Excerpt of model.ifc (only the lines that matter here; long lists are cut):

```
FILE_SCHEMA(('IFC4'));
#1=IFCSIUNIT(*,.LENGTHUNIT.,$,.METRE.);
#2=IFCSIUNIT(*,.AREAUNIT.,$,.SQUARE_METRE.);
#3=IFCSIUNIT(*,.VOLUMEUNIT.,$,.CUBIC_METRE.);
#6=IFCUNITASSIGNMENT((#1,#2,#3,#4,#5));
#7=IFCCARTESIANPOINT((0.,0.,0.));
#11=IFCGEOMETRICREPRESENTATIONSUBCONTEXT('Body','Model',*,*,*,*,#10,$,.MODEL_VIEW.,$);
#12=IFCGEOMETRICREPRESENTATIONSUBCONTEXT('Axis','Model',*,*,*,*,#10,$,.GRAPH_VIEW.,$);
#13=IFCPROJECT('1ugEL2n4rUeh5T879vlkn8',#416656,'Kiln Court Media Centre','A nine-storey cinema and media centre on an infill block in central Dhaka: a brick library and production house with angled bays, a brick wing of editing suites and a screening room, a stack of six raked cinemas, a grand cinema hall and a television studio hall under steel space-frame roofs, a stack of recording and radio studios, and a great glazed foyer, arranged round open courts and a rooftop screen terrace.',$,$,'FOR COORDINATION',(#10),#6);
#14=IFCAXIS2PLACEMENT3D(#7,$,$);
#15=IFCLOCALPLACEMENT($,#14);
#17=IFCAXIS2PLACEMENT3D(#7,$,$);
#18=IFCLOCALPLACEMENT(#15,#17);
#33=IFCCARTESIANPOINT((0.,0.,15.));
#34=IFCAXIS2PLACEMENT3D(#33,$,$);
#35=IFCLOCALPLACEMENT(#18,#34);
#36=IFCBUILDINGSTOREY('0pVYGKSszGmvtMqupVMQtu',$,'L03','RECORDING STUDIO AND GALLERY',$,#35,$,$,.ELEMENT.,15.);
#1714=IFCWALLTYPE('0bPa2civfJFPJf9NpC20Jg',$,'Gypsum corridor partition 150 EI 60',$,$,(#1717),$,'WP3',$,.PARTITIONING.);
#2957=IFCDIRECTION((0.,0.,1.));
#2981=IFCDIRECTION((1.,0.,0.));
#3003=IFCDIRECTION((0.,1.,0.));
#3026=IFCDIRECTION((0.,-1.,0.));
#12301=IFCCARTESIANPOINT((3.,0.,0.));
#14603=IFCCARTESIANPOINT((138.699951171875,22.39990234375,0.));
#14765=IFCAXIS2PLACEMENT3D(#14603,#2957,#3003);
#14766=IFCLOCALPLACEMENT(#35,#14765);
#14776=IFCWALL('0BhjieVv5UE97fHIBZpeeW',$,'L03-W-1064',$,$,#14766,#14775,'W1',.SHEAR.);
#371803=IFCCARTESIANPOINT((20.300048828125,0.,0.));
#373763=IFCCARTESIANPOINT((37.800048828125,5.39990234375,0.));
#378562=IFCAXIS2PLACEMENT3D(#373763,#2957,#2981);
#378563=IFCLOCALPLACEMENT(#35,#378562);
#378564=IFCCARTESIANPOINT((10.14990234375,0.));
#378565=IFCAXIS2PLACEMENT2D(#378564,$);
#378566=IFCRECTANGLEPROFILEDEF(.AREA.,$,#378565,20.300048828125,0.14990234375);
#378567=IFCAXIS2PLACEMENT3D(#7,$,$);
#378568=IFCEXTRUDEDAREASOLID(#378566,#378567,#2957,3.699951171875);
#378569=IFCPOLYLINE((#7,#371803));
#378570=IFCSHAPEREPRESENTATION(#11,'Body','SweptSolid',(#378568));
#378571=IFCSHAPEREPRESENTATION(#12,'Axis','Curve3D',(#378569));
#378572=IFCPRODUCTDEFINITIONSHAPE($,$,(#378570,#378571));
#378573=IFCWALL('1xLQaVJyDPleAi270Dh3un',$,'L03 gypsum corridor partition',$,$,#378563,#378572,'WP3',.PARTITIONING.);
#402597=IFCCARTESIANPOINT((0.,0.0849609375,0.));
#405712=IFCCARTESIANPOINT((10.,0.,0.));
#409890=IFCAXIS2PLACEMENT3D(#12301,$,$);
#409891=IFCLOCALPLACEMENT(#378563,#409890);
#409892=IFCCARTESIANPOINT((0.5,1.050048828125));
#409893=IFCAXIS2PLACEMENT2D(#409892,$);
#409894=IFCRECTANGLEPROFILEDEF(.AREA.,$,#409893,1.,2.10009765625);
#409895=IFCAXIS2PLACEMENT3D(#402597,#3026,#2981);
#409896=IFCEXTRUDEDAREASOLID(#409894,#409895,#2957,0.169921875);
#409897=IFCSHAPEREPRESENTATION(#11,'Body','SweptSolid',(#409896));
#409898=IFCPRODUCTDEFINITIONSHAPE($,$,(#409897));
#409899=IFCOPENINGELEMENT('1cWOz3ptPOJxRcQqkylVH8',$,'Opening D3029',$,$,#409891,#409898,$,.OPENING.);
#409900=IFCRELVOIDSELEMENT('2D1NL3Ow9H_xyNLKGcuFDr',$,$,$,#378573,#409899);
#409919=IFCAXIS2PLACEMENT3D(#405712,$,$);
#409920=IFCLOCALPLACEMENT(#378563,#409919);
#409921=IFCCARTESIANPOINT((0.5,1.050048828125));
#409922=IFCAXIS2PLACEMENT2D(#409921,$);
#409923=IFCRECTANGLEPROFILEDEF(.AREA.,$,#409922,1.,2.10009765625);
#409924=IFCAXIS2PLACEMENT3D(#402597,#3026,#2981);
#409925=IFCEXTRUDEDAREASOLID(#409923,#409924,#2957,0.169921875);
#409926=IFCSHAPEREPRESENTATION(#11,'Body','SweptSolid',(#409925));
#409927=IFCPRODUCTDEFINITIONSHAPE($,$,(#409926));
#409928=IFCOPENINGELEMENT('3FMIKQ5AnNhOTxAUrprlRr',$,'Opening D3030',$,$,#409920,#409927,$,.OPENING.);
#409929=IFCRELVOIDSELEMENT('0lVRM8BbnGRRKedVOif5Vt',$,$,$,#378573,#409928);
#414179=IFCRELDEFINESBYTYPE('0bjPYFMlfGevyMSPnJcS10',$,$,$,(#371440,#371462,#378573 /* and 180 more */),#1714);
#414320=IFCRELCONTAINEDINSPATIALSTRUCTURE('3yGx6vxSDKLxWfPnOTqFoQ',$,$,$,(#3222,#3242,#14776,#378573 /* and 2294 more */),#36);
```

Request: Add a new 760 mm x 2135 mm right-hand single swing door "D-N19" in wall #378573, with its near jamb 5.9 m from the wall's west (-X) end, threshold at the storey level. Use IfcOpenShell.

```python
import numpy as np
import ifcopenshell
import ifcopenshell.api.feature
import ifcopenshell.api.geometry
import ifcopenshell.api.root
import ifcopenshell.api.spatial
import ifcopenshell.geom
import ifcopenshell.util.element
import ifcopenshell.util.placement
import ifcopenshell.util.representation
import ifcopenshell.util.shape
import ifcopenshell.util.unit

model = ifcopenshell.open("model.ifc")
unit_scale = ifcopenshell.util.unit.calculate_unit_scale(model)
settings = ifcopenshell.geom.settings()


def volume(element):
    """Net volume in cubic metres, openings subtracted."""
    shape = ifcopenshell.geom.create_shape(settings, element)
    return ifcopenshell.util.shape.get_volume(shape.geometry)


wall = model.by_guid("1xLQaVJyDPleAi270Dh3un")
storey = ifcopenshell.util.element.get_container(wall, ifc_class="IfcBuildingStorey")
context = ifcopenshell.util.representation.get_context(model, "Model", "Body", "MODEL_VIEW")
before = volume(wall)

width, height, from_end, sill = 0.76, 2.135, 5.9, 0.0  # metres

# The wall runs along its own X axis, and the end named is its -X end.
wall_shape = ifcopenshell.geom.create_shape(settings, wall)
x, y, z = ifcopenshell.util.shape.get_vertices(wall_shape.geometry).T
start = x.min() + from_end
face, thickness = float(y.min()), float(y.max() - y.min())
wall_matrix = ifcopenshell.util.placement.get_local_placement(wall.ObjectPlacement)
level = ifcopenshell.util.placement.get_local_placement(storey.ObjectPlacement)[2, 3]


def in_wall(x, y):
    """Placement at x, y metres in the wall's axes, at sill height."""
    matrix = wall_matrix.copy()
    matrix[:, 3] = wall_matrix @ np.array([x / unit_scale, y / unit_scale, 0.0, 1.0])
    matrix[2, 3] = level + sill / unit_scale
    return matrix


# Opening: a box that overshoots both wall faces by 50 mm.
opening = ifcopenshell.api.root.create_entity(model, ifc_class="IfcOpeningElement", predefined_type="OPENING")
box = ifcopenshell.api.geometry.add_wall_representation(
    model, context=context, length=width, height=height, thickness=thickness + 0.1
)
ifcopenshell.api.geometry.assign_representation(model, product=opening, representation=box)
ifcopenshell.api.geometry.edit_object_placement(model, product=opening, matrix=in_wall(start, face - 0.05), is_si=False)
ifcopenshell.api.feature.add_feature(model, feature=opening, element=wall)

door = ifcopenshell.api.root.create_entity(model, ifc_class="IfcDoor", name="D-N19", predefined_type="DOOR")
door.OverallWidth, door.OverallHeight = width / unit_scale, height / unit_scale
door.OperationType = "SINGLE_SWING_RIGHT"
body = ifcopenshell.api.geometry.add_door_representation(
    model,
    context=context,
    overall_width=door.OverallWidth,
    overall_height=door.OverallHeight,
    operation_type="SINGLE_SWING_RIGHT",
    lining_properties={"LiningDepth": thickness / unit_scale, "ThresholdDepth": thickness / unit_scale},
)
ifcopenshell.api.geometry.assign_representation(model, product=door, representation=body)
ifcopenshell.api.spatial.assign_container(model, products=[door], relating_structure=storey)
ifcopenshell.api.feature.add_filling(model, opening=opening, element=door)

# The lining spans the wall, so the door starts at the wall face.
ifcopenshell.api.geometry.edit_object_placement(model, product=door, matrix=in_wall(start, face), is_si=False)

after = volume(wall)

print(f"wall volume {before:.3f} -> {after:.3f} m3")

model.write("model_edited.ifc")
```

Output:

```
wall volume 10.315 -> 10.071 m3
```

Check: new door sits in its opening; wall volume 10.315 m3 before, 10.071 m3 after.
